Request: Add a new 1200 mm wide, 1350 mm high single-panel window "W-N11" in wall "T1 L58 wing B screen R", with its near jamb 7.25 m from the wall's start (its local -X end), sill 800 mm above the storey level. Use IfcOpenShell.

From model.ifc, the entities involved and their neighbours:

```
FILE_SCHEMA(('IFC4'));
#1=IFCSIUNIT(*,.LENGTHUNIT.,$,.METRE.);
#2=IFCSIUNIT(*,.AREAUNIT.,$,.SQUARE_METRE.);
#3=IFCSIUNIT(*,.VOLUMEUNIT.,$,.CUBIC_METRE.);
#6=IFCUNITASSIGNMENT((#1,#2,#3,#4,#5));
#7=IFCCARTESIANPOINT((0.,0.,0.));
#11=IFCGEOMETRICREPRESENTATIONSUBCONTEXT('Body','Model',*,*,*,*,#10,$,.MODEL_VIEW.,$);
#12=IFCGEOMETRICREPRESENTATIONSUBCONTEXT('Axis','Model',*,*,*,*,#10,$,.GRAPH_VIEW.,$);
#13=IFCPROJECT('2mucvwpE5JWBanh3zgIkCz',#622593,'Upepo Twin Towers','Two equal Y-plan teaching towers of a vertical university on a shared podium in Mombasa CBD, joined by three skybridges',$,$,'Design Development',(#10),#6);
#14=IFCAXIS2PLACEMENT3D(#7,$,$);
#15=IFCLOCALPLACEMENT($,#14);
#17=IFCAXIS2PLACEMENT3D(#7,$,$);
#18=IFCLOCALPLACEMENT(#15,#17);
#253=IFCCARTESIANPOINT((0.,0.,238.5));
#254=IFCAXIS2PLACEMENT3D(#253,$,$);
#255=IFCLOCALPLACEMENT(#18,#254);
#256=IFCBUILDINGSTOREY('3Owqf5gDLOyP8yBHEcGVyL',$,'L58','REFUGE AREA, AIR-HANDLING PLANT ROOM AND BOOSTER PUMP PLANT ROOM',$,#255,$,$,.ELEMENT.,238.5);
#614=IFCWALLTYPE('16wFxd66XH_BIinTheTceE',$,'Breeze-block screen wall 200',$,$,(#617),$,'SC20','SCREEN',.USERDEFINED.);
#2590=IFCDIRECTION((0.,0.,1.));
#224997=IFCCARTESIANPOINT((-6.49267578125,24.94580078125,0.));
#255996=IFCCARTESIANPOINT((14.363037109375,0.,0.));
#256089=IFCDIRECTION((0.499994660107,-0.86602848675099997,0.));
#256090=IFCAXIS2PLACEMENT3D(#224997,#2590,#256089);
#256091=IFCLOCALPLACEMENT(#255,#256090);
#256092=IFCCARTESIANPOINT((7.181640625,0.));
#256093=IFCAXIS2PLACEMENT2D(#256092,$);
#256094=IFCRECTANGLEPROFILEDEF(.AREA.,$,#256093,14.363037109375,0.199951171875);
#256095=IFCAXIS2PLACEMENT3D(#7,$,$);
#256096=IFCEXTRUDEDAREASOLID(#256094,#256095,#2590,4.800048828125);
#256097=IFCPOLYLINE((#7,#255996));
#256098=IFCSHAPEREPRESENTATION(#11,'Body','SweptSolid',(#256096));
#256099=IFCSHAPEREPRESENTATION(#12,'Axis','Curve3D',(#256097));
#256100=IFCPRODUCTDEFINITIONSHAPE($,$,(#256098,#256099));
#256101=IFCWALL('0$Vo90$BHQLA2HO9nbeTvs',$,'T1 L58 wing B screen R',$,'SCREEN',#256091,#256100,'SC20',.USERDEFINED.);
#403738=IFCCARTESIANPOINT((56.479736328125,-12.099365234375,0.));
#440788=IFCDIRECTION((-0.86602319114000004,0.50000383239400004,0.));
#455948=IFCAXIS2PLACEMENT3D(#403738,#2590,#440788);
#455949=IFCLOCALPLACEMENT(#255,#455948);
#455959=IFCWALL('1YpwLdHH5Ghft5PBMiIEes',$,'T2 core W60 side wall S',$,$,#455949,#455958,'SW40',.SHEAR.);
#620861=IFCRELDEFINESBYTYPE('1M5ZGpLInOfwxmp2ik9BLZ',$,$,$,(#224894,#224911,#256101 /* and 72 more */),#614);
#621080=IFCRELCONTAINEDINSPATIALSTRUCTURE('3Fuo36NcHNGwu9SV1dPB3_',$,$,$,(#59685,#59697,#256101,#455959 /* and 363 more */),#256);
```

```python
import numpy as np
import ifcopenshell
import ifcopenshell.api.feature
import ifcopenshell.api.geometry
import ifcopenshell.api.root
import ifcopenshell.api.spatial
import ifcopenshell.geom
import ifcopenshell.util.element
import ifcopenshell.util.placement
import ifcopenshell.util.representation
import ifcopenshell.util.shape
import ifcopenshell.util.unit

model = ifcopenshell.open("model.ifc")
unit_scale = ifcopenshell.util.unit.calculate_unit_scale(model)
settings = ifcopenshell.geom.settings()


def volume(element):
    """Net volume in cubic metres, openings subtracted."""
    shape = ifcopenshell.geom.create_shape(settings, element)
    return ifcopenshell.util.shape.get_volume(shape.geometry)


wall = model.by_guid("0$Vo90$BHQLA2HO9nbeTvs")
storey = ifcopenshell.util.element.get_container(wall, ifc_class="IfcBuildingStorey")
context = ifcopenshell.util.representation.get_context(model, "Model", "Body", "MODEL_VIEW")
before = volume(wall)

width, height, from_end, sill = 1.2, 1.35, 7.25, 0.8  # metres

# The wall runs along its own X axis, and the end named is its -X end.
wall_shape = ifcopenshell.geom.create_shape(settings, wall)
x, y, z = ifcopenshell.util.shape.get_vertices(wall_shape.geometry).T
start = x.min() + from_end
face, thickness = float(y.min()), float(y.max() - y.min())
wall_matrix = ifcopenshell.util.placement.get_local_placement(wall.ObjectPlacement)
level = ifcopenshell.util.placement.get_local_placement(storey.ObjectPlacement)[2, 3]


def in_wall(x, y):
    """Placement at x, y metres in the wall's axes, at sill height."""
    matrix = wall_matrix.copy()
    matrix[:, 3] = wall_matrix @ np.array([x / unit_scale, y / unit_scale, 0.0, 1.0])
    matrix[2, 3] = level + sill / unit_scale
    return matrix


# Opening: a box that overshoots both wall faces by 50 mm.
opening = ifcopenshell.api.root.create_entity(model, ifc_class="IfcOpeningElement", predefined_type="OPENING")
box = ifcopenshell.api.geometry.add_wall_representation(
    model, context=context, length=width, height=height, thickness=thickness + 0.1
)
ifcopenshell.api.geometry.assign_representation(model, product=opening, representation=box)
ifcopenshell.api.geometry.edit_object_placement(model, product=opening, matrix=in_wall(start, face - 0.05), is_si=False)
ifcopenshell.api.feature.add_feature(model, feature=opening, element=wall)

window = ifcopenshell.api.root.create_entity(model, ifc_class="IfcWindow", name="W-N11", predefined_type="WINDOW")
window.OverallWidth, window.OverallHeight = width / unit_scale, height / unit_scale
window.PartitioningType = "SINGLE_PANEL"
body = ifcopenshell.api.geometry.add_window_representation(
    model,
    context=context,
    overall_width=window.OverallWidth,
    overall_height=window.OverallHeight,
    partition_type="SINGLE_PANEL",
)
ifcopenshell.api.geometry.assign_representation(model, product=window, representation=body)
ifcopenshell.api.spatial.assign_container(model, products=[window], relating_structure=storey)
ifcopenshell.api.feature.add_filling(model, opening=opening, element=window)

# Centre the window in the wall's thickness.
ifcopenshell.api.geometry.edit_object_placement(model, product=window, matrix=in_wall(start, face), is_si=False)
window_shape = ifcopenshell.geom.create_shape(settings, window)
depth = ifcopenshell.util.shape.get_vertices(window_shape.geometry)[:, 1]
offset = face + thickness / 2 - (depth.min() + depth.max()) / 2
ifcopenshell.api.geometry.edit_object_placement(model, product=window, matrix=in_wall(start, offset), is_si=False)

after = volume(wall)

print(f"wall volume {before:.3f} -> {after:.3f} m3")

model.write("model_v2.ifc")
```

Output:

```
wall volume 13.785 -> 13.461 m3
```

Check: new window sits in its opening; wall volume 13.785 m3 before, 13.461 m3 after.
